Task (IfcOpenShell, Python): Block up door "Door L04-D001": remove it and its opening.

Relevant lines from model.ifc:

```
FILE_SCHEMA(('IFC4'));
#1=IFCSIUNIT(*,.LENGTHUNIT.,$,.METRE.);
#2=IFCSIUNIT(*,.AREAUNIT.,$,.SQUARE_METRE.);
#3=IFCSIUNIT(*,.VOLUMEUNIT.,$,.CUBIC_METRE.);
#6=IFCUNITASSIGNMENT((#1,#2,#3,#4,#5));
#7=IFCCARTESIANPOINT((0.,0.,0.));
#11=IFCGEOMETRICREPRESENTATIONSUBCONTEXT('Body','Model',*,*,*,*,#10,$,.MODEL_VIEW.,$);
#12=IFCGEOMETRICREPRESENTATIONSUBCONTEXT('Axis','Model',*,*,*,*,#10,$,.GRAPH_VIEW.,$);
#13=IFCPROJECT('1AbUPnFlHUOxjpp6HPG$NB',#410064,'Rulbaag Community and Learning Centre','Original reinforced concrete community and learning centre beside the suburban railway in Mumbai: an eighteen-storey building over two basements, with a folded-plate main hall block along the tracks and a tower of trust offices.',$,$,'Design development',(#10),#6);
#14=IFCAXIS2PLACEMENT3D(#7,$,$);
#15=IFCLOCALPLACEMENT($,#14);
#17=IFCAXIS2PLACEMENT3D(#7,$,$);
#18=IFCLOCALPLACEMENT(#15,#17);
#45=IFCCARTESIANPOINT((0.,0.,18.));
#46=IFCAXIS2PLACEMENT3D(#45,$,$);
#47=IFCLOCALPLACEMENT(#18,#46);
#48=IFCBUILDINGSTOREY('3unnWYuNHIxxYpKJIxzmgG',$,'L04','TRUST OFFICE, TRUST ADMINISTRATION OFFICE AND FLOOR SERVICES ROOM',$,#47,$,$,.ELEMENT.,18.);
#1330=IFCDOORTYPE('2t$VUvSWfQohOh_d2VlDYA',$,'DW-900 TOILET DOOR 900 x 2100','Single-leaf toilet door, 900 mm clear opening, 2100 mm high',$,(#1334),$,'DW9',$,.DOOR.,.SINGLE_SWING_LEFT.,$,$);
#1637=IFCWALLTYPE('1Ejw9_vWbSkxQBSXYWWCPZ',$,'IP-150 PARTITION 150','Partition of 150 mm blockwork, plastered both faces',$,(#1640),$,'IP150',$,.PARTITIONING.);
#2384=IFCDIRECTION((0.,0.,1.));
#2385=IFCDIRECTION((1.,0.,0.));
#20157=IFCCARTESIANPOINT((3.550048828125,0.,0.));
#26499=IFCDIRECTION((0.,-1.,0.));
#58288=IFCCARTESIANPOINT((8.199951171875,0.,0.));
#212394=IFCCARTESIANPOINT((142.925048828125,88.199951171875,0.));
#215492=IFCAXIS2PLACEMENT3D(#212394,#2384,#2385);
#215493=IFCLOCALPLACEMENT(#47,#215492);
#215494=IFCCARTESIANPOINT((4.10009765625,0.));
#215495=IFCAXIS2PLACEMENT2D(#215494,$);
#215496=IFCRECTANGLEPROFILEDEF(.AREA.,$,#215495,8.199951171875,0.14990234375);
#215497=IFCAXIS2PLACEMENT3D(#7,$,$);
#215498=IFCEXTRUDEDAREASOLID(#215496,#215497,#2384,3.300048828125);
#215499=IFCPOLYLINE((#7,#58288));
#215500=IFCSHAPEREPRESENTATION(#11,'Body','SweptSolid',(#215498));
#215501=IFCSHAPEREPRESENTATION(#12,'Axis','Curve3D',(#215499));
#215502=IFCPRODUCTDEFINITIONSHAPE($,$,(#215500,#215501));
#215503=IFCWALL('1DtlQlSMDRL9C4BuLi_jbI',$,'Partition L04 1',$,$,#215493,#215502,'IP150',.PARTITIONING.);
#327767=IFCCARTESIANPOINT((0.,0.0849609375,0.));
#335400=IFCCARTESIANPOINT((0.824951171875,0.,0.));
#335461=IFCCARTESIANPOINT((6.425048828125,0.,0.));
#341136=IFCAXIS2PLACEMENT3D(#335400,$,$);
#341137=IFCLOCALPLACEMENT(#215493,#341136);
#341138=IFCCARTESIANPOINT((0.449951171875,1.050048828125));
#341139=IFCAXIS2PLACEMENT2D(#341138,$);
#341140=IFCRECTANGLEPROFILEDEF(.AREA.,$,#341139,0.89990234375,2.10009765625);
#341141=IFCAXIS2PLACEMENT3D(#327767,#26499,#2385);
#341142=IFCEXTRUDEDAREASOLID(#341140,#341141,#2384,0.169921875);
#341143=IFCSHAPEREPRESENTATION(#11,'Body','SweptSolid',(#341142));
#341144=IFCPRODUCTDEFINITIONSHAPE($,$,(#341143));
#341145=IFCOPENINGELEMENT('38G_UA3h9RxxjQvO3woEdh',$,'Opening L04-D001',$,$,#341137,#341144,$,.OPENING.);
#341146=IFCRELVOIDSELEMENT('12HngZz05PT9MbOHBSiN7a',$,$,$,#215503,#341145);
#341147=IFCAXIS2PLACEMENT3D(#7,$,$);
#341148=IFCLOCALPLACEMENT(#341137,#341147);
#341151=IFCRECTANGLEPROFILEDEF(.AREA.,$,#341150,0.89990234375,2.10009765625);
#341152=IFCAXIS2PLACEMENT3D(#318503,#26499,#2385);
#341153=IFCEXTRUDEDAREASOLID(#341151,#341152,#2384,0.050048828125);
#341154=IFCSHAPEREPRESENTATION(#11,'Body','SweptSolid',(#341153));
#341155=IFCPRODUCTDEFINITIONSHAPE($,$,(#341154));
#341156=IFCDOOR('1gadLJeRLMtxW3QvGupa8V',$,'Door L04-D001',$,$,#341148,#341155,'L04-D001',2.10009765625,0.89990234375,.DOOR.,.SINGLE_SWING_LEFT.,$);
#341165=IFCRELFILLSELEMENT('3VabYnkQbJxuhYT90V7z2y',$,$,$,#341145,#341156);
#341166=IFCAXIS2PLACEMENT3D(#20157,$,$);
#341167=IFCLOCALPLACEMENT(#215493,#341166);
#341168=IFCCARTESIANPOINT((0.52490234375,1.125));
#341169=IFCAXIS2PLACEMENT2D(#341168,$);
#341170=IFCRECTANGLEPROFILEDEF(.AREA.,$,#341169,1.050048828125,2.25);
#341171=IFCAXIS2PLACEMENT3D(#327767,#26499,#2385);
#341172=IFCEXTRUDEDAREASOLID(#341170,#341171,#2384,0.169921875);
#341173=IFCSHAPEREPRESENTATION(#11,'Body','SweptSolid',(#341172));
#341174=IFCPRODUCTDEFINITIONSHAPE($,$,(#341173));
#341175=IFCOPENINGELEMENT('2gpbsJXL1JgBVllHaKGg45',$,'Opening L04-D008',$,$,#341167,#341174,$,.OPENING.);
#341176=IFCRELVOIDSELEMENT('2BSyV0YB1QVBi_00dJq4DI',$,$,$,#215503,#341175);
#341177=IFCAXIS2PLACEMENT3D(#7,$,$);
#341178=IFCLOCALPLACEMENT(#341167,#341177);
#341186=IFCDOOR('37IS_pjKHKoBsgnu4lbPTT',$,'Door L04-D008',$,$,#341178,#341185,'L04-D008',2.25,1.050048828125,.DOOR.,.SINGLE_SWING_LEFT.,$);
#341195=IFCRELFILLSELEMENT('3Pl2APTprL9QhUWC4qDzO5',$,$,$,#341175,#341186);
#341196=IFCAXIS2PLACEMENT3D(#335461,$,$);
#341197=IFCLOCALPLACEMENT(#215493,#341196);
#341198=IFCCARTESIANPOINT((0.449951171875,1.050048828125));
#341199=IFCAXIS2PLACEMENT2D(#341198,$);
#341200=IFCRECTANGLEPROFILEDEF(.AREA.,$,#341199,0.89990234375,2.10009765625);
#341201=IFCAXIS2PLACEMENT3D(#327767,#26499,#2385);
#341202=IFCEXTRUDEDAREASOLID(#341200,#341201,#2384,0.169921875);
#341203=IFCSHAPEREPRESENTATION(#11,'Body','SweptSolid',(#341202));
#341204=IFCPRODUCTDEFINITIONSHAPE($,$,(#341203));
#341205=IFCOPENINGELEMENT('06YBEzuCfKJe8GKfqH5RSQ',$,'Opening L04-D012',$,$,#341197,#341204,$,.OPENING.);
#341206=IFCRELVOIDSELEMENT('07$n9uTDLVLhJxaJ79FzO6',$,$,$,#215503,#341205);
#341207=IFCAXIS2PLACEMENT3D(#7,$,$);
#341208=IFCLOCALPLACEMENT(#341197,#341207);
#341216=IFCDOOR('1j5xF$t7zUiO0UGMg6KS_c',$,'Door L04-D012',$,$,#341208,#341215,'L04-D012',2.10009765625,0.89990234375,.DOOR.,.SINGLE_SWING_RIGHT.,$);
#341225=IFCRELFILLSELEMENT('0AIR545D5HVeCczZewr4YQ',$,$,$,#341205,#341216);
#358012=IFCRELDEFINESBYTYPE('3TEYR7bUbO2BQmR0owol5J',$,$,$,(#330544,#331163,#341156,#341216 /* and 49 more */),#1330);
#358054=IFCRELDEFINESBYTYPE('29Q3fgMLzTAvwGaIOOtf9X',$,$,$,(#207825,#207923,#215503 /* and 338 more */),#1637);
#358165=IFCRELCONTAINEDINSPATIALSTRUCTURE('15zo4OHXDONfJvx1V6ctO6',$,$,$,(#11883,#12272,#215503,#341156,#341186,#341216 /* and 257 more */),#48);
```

```python
import ifcopenshell
import ifcopenshell.api.feature
import ifcopenshell.api.root
import ifcopenshell.geom
import ifcopenshell.util.shape

model = ifcopenshell.open("model.ifc")
settings = ifcopenshell.geom.settings()


def volume(element):
    """Net volume in cubic metres, openings subtracted."""
    shape = ifcopenshell.geom.create_shape(settings, element)
    return ifcopenshell.util.shape.get_volume(shape.geometry)


door = model.by_guid("1gadLJeRLMtxW3QvGupa8V")
opening = door.FillsVoids[0].RelatingOpeningElement
wall = opening.VoidsElements[0].RelatingBuildingElement
before = volume(wall)

ifcopenshell.api.root.remove_product(model, product=door)
ifcopenshell.api.feature.remove_feature(model, feature=opening)

after = volume(wall)

print(f"wall volume {before:.3f} -> {after:.3f} m3")

model.write("model-out.ifc")
```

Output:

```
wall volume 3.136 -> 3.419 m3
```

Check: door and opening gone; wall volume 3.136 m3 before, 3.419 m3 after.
